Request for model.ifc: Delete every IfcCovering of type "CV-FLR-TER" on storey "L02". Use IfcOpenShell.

First a look at what the model holds.

```python
import ifcopenshell
import ifcopenshell.util.element

model = ifcopenshell.open("model.ifc")
print(model.schema)
storey = next(s for s in model.by_type("IfcBuildingStorey") if s.Name == "L02")
coverings = [e for e in ifcopenshell.util.element.get_decomposition(storey) if e.is_a("IfcCovering")]
seen = {}
for e in coverings:
    element_type = ifcopenshell.util.element.get_type(e)
    name = element_type.Name if element_type not in (None, e) else None
    seen[name] = seen.get(name, 0) + 1
for name, count in sorted(seen.items(), key=str):
    print(count, "x", name)
```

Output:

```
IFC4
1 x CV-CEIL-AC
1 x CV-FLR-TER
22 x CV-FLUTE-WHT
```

```python
import ifcopenshell
import ifcopenshell.api.root
import ifcopenshell.util.element

model = ifcopenshell.open("model.ifc")

storey = next(s for s in model.by_type("IfcBuildingStorey") if s.Name == "L02")
coverings = [e for e in ifcopenshell.util.element.get_decomposition(storey) if e.is_a("IfcCovering")]
targets = [e for e in coverings if (t := ifcopenshell.util.element.get_type(e)) not in (None, e) and t.Name == "CV-FLR-TER"]

for e in targets:
    ifcopenshell.api.root.remove_product(model, product=e)
print(len(targets), "removed")

model.write("model_v2.ifc")
```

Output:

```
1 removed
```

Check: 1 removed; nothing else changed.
